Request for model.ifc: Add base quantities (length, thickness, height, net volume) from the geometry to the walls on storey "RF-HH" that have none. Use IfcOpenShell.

First a look at what the model holds.

```python
import ifcopenshell
import ifcopenshell.util.element
import ifcopenshell.util.unit

model = ifcopenshell.open("model.ifc")
print(model.schema)
for unit_type in ("LENGTHUNIT", "AREAUNIT", "VOLUMEUNIT"):
    print(unit_type, ifcopenshell.util.unit.calculate_unit_scale(model, unit_type))
storey = next(s for s in model.by_type("IfcBuildingStorey") if s.Name == "RF-HH")
walls = [e for e in ifcopenshell.util.element.get_decomposition(storey) if e.is_a("IfcWall")]
for e in sorted(walls, key=lambda e: e.id()):
    print(e.id(), e.is_a(), e.Name, list(ifcopenshell.util.element.get_psets(e, qtos_only=True)), sep=" | ")
```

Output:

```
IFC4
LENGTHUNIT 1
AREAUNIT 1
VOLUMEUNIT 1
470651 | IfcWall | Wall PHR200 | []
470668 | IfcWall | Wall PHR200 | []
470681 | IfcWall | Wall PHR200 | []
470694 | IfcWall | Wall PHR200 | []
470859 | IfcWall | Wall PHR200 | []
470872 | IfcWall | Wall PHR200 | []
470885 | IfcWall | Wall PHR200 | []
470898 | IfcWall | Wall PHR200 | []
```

```python
import ifcopenshell
import ifcopenshell.api.pset
import ifcopenshell.geom
import ifcopenshell.util.element
import ifcopenshell.util.shape
import ifcopenshell.util.unit

model = ifcopenshell.open("model.ifc")
unit_scale = ifcopenshell.util.unit.calculate_unit_scale(model)
volume_scale = ifcopenshell.util.unit.calculate_unit_scale(model, "VOLUMEUNIT")
settings = ifcopenshell.geom.settings()

storey = next(s for s in model.by_type("IfcBuildingStorey") if s.Name == "RF-HH")
walls = [e for e in ifcopenshell.util.element.get_decomposition(storey) if e.is_a("IfcWall")]

for e in sorted(walls, key=lambda e: e.id()):
    if ifcopenshell.util.element.get_psets(e, qtos_only=True, should_inherit=False):
        continue
    # Geometry comes back in metres, in the element's own axes.
    shape = ifcopenshell.geom.create_shape(settings, e)
    values = {
        "Length": ifcopenshell.util.shape.get_x(shape.geometry) / unit_scale,
        "Width": ifcopenshell.util.shape.get_y(shape.geometry) / unit_scale,
        "Height": ifcopenshell.util.shape.get_z(shape.geometry) / unit_scale,
        "NetVolume": ifcopenshell.util.shape.get_volume(shape.geometry) / volume_scale,
    }
    qto = ifcopenshell.api.pset.add_qto(model, product=e, name="Qto_WallBaseQuantities")
    ifcopenshell.api.pset.edit_qto(model, qto=qto, properties=values)
    print(e.id(), {k: round(v, 3) for k, v in values.items()})

model.write("model_updated.ifc")
```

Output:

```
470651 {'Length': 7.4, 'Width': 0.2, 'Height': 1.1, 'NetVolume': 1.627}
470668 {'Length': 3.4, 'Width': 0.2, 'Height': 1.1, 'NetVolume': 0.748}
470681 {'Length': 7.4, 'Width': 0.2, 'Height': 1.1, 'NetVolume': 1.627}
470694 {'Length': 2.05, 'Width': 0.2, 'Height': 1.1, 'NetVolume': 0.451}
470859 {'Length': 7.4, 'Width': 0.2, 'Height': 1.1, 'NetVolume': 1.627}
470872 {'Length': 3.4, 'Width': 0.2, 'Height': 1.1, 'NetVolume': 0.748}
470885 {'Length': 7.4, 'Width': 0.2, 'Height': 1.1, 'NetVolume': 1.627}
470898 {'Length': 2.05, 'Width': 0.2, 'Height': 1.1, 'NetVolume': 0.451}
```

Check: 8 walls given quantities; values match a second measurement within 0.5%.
